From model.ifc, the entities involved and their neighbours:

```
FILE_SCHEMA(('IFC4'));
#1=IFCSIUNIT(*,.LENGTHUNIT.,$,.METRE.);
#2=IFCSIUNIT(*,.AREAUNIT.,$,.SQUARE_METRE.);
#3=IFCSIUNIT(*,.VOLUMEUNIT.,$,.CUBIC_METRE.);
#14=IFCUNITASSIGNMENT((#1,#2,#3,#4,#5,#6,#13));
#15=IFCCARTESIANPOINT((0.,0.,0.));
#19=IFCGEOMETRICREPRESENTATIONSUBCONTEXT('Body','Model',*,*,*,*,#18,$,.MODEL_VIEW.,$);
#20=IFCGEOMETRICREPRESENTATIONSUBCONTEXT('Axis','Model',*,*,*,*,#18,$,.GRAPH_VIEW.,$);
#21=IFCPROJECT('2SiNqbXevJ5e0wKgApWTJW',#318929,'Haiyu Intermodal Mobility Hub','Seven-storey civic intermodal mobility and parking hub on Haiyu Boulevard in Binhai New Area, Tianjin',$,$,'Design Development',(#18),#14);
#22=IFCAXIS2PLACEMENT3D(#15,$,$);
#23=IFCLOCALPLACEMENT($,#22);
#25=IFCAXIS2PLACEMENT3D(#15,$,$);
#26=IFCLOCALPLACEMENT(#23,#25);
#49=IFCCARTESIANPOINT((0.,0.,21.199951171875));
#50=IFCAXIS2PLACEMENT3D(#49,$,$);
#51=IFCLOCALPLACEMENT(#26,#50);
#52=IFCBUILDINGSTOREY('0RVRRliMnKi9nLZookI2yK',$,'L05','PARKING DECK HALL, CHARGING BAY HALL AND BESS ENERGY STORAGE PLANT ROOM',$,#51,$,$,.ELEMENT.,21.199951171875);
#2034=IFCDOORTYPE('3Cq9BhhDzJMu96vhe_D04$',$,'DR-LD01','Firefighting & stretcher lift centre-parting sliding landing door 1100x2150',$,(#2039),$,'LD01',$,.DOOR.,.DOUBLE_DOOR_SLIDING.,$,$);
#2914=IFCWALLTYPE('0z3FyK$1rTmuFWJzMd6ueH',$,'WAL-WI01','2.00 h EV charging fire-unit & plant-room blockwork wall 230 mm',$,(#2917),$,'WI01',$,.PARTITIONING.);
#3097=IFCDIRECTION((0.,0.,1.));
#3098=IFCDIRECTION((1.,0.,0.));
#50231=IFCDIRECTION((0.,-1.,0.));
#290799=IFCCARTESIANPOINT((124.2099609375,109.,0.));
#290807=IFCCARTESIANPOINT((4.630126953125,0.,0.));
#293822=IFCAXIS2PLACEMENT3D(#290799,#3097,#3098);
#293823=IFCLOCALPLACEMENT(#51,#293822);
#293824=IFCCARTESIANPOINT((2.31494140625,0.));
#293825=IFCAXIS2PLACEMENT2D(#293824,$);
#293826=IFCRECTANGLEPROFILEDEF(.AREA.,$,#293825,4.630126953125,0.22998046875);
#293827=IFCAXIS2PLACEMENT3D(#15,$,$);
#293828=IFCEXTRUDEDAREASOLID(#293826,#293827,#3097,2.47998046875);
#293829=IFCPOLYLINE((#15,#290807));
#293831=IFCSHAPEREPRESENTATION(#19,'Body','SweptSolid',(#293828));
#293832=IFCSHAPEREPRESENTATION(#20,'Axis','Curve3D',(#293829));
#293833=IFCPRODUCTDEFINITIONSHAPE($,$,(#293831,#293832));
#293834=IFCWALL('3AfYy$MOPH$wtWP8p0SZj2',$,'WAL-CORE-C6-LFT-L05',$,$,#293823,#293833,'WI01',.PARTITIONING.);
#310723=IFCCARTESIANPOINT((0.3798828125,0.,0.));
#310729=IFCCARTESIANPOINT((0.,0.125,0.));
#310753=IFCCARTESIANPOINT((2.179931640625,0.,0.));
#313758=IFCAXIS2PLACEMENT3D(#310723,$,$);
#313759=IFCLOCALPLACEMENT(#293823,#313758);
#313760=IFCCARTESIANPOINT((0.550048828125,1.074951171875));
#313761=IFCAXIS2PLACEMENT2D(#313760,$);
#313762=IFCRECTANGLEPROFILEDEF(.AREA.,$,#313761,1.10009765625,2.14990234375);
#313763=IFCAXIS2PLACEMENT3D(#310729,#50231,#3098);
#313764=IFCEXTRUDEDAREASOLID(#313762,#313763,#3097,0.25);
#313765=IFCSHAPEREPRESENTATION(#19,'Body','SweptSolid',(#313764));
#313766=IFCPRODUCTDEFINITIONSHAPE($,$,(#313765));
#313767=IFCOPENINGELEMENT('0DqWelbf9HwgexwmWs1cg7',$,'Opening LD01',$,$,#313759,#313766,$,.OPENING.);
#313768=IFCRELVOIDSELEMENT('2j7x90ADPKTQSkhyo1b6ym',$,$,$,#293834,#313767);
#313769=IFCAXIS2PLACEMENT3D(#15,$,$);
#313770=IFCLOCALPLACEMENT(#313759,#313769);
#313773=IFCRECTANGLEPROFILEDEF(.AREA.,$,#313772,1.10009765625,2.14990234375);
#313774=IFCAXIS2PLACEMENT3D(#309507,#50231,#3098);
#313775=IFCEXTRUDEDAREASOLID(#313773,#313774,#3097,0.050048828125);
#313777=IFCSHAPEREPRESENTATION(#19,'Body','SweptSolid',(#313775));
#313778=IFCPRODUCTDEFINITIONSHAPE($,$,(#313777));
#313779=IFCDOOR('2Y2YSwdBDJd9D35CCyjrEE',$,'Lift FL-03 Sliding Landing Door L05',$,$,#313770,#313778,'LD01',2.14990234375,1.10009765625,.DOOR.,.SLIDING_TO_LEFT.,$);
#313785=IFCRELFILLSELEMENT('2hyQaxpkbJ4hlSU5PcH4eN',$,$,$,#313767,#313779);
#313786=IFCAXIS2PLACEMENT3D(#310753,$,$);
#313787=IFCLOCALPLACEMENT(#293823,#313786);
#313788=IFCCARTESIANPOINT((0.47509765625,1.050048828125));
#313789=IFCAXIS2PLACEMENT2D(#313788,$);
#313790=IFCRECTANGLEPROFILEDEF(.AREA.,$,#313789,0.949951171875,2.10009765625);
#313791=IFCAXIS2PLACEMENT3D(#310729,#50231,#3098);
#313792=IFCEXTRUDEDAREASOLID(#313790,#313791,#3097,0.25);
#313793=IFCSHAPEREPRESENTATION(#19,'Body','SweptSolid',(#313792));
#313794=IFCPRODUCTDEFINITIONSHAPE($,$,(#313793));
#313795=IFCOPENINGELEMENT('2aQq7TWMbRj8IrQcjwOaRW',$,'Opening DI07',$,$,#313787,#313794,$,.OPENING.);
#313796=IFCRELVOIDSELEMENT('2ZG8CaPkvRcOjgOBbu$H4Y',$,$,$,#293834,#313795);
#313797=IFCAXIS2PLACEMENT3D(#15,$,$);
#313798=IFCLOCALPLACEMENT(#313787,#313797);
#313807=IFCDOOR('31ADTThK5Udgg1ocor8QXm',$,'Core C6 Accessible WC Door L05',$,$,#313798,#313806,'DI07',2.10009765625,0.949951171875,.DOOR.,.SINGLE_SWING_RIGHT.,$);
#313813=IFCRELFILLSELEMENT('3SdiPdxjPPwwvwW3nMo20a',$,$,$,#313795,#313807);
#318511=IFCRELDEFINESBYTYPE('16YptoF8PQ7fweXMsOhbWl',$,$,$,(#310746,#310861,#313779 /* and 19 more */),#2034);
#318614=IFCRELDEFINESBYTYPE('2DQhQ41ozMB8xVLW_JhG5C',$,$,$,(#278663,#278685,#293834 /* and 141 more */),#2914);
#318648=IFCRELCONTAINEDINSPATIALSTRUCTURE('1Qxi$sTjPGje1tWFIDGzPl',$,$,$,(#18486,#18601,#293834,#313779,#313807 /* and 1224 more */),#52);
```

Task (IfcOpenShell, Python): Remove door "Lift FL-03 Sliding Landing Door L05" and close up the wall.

```python
import ifcopenshell
import ifcopenshell.api.feature
import ifcopenshell.api.root
import ifcopenshell.geom
import ifcopenshell.util.shape

model = ifcopenshell.open("model.ifc")
settings = ifcopenshell.geom.settings()


def volume(element):
    """Net volume in cubic metres, openings subtracted."""
    shape = ifcopenshell.geom.create_shape(settings, element)
    return ifcopenshell.util.shape.get_volume(shape.geometry)


door = model.by_guid("2Y2YSwdBDJd9D35CCyjrEE")
opening = door.FillsVoids[0].RelatingOpeningElement
wall = opening.VoidsElements[0].RelatingBuildingElement
before = volume(wall)

ifcopenshell.api.root.remove_product(model, product=door)
ifcopenshell.api.feature.remove_feature(model, feature=opening)

after = volume(wall)

print(f"wall volume {before:.3f} -> {after:.3f} m3")

model.write("model-out.ifc")
```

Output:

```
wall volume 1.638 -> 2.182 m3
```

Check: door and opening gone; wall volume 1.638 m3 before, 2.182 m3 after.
